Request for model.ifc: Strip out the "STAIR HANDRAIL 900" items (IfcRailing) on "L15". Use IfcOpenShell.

First a look at what the model holds.

```python
import ifcopenshell
import ifcopenshell.util.element

model = ifcopenshell.open("model.ifc")
print(model.schema)
storey = next(s for s in model.by_type("IfcBuildingStorey") if s.Name == "L15")
railings = [e for e in ifcopenshell.util.element.get_decomposition(storey) if e.is_a("IfcRailing")]
seen = {}
for e in railings:
    element_type = ifcopenshell.util.element.get_type(e)
    name = element_type.Name if element_type not in (None, e) else None
    seen[name] = seen.get(name, 0) + 1
for name, count in sorted(seen.items(), key=str):
    print(count, "x", name)
```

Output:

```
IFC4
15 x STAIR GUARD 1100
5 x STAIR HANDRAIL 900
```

```python
import ifcopenshell
import ifcopenshell.api.root
import ifcopenshell.util.element

model = ifcopenshell.open("model.ifc")

storey = next(s for s in model.by_type("IfcBuildingStorey") if s.Name == "L15")
railings = [e for e in ifcopenshell.util.element.get_decomposition(storey) if e.is_a("IfcRailing")]
targets = [e for e in railings if (t := ifcopenshell.util.element.get_type(e)) not in (None, e) and t.Name == "STAIR HANDRAIL 900"]

for e in targets:
    ifcopenshell.api.root.remove_product(model, product=e)
print(len(targets), "removed")

model.write("model_edited.ifc")
```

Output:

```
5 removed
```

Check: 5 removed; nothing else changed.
